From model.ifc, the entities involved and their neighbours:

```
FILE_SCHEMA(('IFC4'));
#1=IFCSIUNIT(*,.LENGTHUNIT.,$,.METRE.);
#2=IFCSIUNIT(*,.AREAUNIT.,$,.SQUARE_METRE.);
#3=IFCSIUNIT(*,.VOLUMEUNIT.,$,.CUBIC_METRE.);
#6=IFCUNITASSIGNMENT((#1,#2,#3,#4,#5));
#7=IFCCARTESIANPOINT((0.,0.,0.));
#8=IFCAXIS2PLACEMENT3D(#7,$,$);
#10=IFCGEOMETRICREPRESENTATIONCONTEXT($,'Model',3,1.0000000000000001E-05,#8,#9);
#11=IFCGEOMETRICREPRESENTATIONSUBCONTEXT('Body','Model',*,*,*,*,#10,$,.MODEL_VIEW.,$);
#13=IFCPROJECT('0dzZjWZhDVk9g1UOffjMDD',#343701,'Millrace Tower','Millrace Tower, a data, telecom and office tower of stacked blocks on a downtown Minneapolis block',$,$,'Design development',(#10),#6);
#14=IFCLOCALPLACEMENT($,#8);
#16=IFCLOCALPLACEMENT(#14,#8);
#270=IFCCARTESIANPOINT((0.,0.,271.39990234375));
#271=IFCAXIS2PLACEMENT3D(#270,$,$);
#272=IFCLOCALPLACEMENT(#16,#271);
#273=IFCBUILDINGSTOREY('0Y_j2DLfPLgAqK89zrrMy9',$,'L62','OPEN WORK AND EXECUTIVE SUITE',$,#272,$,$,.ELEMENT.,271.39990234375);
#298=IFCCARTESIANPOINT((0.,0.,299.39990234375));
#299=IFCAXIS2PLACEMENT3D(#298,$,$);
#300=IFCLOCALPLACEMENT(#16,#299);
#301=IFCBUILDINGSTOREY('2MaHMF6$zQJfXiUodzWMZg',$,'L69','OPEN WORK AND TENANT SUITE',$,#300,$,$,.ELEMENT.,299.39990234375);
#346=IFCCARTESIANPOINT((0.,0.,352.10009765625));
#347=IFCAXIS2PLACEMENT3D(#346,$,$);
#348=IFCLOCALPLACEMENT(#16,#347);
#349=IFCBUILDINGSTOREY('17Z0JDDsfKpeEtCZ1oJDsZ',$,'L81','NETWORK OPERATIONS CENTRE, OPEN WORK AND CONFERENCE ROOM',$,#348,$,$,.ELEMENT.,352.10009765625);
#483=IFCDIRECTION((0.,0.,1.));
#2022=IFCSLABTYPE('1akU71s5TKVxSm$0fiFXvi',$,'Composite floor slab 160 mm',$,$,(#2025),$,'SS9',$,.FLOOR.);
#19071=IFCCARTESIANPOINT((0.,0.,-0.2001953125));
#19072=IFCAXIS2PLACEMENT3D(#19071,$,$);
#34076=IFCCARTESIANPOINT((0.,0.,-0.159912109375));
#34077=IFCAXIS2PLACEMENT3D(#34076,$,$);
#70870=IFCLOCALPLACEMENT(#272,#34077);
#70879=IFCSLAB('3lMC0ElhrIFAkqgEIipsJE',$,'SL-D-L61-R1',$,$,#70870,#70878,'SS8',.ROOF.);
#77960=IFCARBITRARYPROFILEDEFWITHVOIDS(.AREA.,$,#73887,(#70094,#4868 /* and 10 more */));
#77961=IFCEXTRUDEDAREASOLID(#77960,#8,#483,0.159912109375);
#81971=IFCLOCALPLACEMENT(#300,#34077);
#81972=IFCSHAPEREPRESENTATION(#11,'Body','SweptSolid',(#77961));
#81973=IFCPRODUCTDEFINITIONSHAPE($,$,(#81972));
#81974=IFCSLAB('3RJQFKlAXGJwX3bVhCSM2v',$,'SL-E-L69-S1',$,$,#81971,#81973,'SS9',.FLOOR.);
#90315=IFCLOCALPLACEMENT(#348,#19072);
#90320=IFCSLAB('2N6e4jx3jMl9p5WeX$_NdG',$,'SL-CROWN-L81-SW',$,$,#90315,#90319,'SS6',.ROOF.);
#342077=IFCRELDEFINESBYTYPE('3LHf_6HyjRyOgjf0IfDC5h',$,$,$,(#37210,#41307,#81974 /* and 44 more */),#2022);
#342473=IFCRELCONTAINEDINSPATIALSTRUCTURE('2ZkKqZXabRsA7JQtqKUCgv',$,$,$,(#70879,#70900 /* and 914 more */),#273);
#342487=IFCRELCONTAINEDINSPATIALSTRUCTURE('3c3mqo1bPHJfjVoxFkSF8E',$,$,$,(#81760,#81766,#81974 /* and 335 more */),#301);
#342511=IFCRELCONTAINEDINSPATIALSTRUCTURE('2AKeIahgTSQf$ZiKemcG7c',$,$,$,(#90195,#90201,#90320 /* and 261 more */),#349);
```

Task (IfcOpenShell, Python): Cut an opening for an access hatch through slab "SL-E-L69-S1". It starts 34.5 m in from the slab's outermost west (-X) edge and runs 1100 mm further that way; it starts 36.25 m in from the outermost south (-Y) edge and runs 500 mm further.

```python
import numpy as np
import ifcopenshell
import ifcopenshell.api.feature
import ifcopenshell.api.geometry
import ifcopenshell.api.root
import ifcopenshell.geom
import ifcopenshell.util.placement
import ifcopenshell.util.representation
import ifcopenshell.util.shape
import ifcopenshell.util.unit

model = ifcopenshell.open("model.ifc")
unit_scale = ifcopenshell.util.unit.calculate_unit_scale(model)
settings = ifcopenshell.geom.settings()


def volume(element):
    """Net volume in cubic metres, openings subtracted."""
    shape = ifcopenshell.geom.create_shape(settings, element)
    return ifcopenshell.util.shape.get_volume(shape.geometry)


slab = model.by_guid("3RJQFKlAXGJwX3bVhCSM2v")
before = volume(slab)

# Extent in the slab's own axes, in metres. The edges named are its -X and -Y sides.
slab_shape = ifcopenshell.geom.create_shape(settings, slab)
vertices = ifcopenshell.util.shape.get_vertices(slab_shape.geometry)
x_min, y_min, bottom = vertices.min(axis=0)
top = vertices[:, 2].max()

opening = ifcopenshell.api.root.create_entity(model, ifc_class="IfcOpeningElement", name="Access hatch opening", predefined_type="OPENING")
context = ifcopenshell.util.representation.get_context(model, "Model", "Body", "MODEL_VIEW")
width, depth = 1.1, 0.5
outline = [(0.0, 0.0), (width, 0.0), (width, depth), (0.0, depth), (0.0, 0.0)]
# Overshoot both faces by 50 mm so the cut is clean.
shape = ifcopenshell.api.geometry.add_slab_representation(
    model, context=context, depth=top - bottom + 0.1, polyline=outline
)
ifcopenshell.api.geometry.assign_representation(model, product=opening, representation=shape)

matrix = ifcopenshell.util.placement.get_local_placement(slab.ObjectPlacement)
matrix[:, 3] = matrix @ np.append(np.array([x_min + 34.5, y_min + 36.25, bottom - 0.05]) / unit_scale, 1.0)
ifcopenshell.api.geometry.edit_object_placement(model, product=opening, matrix=matrix, is_si=False)
ifcopenshell.api.feature.add_feature(model, feature=opening, element=slab)

after = volume(slab)

print(f"slab volume {before:.3f} -> {after:.3f} m3")

model.write("model_edited.ifc")
```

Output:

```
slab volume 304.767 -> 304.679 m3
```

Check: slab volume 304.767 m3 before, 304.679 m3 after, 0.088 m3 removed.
